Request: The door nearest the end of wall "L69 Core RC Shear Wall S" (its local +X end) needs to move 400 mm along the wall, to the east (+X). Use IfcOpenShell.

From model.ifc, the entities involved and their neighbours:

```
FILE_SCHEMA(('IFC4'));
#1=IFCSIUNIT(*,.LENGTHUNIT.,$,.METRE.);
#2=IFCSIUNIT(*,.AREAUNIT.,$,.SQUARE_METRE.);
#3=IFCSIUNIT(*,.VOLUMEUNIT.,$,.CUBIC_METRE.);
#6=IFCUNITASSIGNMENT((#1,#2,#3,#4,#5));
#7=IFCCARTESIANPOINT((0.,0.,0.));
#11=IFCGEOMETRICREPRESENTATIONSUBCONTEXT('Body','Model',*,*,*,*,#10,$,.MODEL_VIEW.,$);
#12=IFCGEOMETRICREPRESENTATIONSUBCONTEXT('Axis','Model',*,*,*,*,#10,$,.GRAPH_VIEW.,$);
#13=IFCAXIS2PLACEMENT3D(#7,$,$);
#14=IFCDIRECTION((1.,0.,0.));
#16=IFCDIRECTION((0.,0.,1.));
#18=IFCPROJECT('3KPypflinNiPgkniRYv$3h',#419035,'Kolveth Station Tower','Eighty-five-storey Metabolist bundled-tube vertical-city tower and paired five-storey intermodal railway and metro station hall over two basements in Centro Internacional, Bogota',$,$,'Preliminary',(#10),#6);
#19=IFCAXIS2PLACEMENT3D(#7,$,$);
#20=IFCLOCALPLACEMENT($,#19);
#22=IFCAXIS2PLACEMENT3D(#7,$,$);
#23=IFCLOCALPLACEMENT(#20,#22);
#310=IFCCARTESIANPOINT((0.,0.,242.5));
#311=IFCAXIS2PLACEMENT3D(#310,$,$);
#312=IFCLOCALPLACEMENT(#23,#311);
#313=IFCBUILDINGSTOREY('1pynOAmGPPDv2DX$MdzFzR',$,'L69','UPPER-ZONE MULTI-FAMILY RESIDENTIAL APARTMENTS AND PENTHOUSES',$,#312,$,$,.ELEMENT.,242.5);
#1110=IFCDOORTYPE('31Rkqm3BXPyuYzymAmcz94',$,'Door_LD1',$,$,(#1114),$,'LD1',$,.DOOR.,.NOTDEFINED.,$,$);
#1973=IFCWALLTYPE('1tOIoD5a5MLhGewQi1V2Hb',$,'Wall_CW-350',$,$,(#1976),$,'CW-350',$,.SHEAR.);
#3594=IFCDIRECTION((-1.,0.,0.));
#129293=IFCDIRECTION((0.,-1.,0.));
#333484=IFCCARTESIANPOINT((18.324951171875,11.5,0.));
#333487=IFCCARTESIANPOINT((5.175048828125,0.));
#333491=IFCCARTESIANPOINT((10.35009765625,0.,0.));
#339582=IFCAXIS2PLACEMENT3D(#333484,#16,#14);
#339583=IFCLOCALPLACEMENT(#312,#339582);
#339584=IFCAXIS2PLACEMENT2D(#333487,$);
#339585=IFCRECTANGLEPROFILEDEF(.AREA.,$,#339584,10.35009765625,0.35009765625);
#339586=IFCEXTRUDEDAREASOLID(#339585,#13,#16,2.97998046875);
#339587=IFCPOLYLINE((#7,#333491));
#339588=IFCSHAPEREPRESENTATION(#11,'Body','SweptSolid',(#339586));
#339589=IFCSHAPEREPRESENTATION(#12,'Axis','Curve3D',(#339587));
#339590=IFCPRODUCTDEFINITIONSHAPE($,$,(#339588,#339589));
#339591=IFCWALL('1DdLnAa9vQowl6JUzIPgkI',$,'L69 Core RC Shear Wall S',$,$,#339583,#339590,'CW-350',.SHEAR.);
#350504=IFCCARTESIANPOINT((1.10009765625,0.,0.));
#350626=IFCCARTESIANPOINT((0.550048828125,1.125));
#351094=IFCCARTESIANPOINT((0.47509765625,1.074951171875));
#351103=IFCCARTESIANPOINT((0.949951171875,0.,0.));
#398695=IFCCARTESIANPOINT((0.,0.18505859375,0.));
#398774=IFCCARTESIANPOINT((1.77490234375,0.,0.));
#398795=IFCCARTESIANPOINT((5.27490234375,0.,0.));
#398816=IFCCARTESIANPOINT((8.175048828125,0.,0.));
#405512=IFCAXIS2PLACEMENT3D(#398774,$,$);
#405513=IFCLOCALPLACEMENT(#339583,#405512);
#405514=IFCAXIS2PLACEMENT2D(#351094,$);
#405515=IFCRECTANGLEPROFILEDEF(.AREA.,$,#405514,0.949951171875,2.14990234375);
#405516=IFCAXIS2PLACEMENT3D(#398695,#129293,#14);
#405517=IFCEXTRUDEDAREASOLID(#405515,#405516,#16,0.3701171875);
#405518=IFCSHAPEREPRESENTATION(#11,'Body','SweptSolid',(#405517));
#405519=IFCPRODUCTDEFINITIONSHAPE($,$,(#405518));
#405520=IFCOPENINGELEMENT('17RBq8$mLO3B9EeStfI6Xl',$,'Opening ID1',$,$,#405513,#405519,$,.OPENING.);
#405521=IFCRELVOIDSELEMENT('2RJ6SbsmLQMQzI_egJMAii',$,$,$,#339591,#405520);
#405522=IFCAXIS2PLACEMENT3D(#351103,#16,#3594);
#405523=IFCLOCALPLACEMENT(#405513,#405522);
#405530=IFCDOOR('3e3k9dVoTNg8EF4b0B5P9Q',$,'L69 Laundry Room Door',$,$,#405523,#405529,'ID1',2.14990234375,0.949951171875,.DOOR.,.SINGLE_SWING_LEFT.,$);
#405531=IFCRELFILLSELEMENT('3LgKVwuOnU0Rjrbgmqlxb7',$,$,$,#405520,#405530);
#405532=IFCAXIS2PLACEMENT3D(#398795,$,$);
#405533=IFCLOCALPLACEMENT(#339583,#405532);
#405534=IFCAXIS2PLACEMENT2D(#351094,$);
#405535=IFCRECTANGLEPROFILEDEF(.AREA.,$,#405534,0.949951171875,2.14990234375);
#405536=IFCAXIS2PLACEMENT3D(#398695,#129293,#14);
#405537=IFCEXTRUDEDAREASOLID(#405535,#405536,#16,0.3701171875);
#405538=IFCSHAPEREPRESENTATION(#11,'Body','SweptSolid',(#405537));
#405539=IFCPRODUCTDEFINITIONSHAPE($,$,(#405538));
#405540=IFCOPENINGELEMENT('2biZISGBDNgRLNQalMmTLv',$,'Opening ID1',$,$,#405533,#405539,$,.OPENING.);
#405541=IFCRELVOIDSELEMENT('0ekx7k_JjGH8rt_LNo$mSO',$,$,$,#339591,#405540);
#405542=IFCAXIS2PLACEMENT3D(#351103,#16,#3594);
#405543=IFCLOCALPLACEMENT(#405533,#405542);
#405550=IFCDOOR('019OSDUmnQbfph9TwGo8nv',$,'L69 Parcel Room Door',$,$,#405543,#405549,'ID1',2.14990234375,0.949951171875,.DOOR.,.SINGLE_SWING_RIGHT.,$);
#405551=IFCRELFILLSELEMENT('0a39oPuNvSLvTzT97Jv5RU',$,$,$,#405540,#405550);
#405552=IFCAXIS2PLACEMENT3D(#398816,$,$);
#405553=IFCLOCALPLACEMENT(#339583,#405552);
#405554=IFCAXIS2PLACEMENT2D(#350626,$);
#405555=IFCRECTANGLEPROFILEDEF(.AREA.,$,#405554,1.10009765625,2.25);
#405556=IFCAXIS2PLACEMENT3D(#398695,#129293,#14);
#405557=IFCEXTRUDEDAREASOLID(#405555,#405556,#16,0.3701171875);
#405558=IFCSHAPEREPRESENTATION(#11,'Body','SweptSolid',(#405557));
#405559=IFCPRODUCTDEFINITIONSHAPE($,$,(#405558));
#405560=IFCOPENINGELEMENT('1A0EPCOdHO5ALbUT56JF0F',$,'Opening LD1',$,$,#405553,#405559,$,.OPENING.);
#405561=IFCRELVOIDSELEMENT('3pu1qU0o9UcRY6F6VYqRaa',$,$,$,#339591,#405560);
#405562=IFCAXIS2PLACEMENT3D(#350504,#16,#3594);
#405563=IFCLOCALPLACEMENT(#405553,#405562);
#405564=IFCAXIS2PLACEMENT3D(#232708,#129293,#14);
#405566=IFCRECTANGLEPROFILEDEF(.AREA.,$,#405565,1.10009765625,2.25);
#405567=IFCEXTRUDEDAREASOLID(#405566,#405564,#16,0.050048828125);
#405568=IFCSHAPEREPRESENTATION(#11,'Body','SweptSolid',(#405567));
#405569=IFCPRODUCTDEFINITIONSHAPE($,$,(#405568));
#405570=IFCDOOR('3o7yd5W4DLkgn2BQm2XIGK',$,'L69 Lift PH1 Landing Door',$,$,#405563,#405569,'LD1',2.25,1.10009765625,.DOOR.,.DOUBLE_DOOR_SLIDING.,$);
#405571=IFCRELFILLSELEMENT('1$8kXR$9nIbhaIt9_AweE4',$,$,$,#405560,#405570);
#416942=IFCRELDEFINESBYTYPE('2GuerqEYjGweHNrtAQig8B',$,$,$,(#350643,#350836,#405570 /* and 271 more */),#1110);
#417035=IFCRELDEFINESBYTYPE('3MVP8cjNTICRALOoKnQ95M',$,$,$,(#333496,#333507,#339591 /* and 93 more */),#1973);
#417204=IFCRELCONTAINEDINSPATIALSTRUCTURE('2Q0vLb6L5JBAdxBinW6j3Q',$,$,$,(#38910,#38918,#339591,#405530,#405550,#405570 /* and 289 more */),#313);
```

```python
import ifcopenshell
import ifcopenshell.api.geometry
import ifcopenshell.util.placement
import ifcopenshell.util.unit

model = ifcopenshell.open("model.ifc")
unit_scale = ifcopenshell.util.unit.calculate_unit_scale(model)

door = model.by_id(405570)
opening = door.FillsVoids[0].RelatingOpeningElement
wall = opening.VoidsElements[0].RelatingBuildingElement

wall_matrix = ifcopenshell.util.placement.get_local_placement(wall.ObjectPlacement)
shift = wall_matrix[:3, 0] * 0.4 / unit_scale
before = ifcopenshell.util.placement.get_local_placement(door.ObjectPlacement)[:3, 3].copy()

# The door is placed relative to its opening, so it follows when the opening moves.
matrix = ifcopenshell.util.placement.get_local_placement(opening.ObjectPlacement)
matrix[:3, 3] += shift
ifcopenshell.api.geometry.edit_object_placement(
    model, product=opening, matrix=matrix, is_si=False, should_transform_children=True
)

after = ifcopenshell.util.placement.get_local_placement(door.ObjectPlacement)[:3, 3]
print("door moved by", (after - before).round(3) + 0.0)

model.write("model-out.ifc")
```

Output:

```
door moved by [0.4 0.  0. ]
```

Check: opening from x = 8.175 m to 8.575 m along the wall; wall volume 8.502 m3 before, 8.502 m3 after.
